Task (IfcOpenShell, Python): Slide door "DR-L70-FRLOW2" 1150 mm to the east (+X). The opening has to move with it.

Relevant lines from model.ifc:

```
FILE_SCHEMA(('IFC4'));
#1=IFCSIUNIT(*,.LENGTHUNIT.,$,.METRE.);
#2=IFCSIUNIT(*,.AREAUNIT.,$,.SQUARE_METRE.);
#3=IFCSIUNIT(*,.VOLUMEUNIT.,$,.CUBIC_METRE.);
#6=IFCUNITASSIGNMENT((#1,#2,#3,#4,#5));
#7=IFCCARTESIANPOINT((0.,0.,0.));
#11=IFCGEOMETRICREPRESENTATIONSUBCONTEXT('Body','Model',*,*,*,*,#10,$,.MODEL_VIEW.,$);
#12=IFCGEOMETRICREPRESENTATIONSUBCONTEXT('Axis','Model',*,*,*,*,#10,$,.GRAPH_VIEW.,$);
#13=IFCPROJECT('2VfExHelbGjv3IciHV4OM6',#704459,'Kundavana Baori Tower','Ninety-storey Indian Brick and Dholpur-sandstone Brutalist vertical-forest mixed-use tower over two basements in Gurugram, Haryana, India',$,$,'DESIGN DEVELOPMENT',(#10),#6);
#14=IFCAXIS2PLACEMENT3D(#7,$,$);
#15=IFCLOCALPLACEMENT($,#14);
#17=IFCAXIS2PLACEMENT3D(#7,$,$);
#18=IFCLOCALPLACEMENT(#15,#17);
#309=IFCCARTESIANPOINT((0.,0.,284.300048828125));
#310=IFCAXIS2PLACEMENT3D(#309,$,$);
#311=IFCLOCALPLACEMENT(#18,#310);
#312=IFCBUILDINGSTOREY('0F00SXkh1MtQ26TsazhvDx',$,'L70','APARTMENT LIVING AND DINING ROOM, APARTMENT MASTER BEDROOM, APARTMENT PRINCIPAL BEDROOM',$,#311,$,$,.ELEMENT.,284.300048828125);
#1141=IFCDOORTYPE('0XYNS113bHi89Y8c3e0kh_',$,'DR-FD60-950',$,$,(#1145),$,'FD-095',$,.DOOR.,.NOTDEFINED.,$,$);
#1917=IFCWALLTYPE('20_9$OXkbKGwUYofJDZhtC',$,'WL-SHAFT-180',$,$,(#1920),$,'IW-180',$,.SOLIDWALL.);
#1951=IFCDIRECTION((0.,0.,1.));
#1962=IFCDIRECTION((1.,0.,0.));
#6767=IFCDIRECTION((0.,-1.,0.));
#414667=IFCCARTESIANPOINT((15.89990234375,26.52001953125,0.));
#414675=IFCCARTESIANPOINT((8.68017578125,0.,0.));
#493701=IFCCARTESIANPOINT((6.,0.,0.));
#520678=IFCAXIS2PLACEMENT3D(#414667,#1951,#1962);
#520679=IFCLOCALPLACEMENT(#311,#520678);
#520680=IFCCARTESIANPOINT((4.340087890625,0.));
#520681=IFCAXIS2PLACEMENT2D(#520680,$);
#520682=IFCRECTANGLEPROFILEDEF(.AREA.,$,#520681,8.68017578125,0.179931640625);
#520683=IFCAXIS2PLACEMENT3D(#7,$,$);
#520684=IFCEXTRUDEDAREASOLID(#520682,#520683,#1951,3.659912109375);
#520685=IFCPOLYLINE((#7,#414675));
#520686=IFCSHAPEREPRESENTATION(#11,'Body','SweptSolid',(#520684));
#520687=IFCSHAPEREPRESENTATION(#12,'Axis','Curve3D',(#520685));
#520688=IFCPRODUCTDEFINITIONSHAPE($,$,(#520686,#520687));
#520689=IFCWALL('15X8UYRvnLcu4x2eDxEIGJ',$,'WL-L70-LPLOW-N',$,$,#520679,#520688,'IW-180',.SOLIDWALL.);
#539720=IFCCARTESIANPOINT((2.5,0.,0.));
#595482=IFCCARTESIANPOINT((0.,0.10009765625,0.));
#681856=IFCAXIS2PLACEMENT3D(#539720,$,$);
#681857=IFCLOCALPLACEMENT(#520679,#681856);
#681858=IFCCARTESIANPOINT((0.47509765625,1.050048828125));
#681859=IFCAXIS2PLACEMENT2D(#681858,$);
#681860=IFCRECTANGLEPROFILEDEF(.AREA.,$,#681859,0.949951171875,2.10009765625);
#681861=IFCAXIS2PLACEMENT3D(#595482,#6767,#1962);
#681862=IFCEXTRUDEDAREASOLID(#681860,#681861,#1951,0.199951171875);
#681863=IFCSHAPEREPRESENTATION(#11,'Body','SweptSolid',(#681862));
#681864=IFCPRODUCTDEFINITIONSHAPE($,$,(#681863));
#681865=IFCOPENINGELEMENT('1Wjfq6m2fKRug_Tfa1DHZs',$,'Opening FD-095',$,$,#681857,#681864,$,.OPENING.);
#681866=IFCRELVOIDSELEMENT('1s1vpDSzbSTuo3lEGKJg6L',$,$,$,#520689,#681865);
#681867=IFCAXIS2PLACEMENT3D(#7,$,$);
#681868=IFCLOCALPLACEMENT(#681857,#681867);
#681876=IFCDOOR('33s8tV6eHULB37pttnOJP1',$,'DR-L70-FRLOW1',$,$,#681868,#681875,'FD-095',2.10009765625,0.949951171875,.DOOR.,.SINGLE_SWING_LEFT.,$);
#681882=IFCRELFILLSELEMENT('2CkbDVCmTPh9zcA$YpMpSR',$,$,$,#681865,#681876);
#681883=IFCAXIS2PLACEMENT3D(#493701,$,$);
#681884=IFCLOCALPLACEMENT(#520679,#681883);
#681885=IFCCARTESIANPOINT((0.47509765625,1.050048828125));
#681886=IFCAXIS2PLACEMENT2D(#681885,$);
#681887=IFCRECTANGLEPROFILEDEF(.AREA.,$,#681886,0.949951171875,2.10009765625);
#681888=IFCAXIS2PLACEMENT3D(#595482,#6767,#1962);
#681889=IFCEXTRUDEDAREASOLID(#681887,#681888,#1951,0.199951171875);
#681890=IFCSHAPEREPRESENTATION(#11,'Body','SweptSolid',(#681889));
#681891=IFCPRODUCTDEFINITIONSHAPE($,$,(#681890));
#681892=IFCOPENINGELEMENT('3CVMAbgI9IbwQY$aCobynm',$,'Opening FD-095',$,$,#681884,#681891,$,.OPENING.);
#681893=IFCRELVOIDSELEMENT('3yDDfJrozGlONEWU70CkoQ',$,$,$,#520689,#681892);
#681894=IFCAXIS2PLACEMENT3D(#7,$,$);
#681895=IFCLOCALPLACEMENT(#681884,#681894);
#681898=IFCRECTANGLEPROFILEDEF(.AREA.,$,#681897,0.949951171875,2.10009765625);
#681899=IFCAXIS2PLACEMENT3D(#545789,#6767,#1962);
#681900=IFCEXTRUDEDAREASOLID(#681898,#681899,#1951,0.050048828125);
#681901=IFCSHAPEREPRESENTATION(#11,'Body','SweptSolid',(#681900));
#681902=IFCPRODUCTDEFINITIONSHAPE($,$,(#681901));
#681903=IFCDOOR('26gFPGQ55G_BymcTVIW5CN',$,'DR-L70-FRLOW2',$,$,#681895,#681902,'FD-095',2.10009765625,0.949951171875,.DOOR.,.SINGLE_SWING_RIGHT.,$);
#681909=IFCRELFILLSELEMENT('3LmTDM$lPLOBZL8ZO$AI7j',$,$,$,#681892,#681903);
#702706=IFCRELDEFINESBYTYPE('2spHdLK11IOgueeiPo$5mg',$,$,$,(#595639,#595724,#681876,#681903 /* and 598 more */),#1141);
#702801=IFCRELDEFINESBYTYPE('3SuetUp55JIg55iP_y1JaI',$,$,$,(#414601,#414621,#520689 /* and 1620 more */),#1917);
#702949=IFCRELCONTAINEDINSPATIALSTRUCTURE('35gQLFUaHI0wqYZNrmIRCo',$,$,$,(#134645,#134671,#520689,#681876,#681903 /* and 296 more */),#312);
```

```python
import ifcopenshell
import ifcopenshell.api.geometry
import ifcopenshell.util.placement
import ifcopenshell.util.unit

model = ifcopenshell.open("model.ifc")
unit_scale = ifcopenshell.util.unit.calculate_unit_scale(model)

door = model.by_guid("26gFPGQ55G_BymcTVIW5CN")
opening = door.FillsVoids[0].RelatingOpeningElement
wall = opening.VoidsElements[0].RelatingBuildingElement

wall_matrix = ifcopenshell.util.placement.get_local_placement(wall.ObjectPlacement)
shift = wall_matrix[:3, 0] * 1.15 / unit_scale
before = ifcopenshell.util.placement.get_local_placement(door.ObjectPlacement)[:3, 3].copy()

# The door is placed relative to its opening, so it follows when the opening moves.
matrix = ifcopenshell.util.placement.get_local_placement(opening.ObjectPlacement)
matrix[:3, 3] += shift
ifcopenshell.api.geometry.edit_object_placement(
    model, product=opening, matrix=matrix, is_si=False, should_transform_children=True
)

after = ifcopenshell.util.placement.get_local_placement(door.ObjectPlacement)[:3, 3]
print("door moved by", (after - before).round(3) + 0.0)

model.write("model_edited.ifc")
```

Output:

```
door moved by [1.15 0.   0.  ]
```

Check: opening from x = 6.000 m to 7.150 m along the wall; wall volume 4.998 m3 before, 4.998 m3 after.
